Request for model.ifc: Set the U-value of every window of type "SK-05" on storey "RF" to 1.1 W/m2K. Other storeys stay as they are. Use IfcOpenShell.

First a look at what the model holds.

```python
import ifcopenshell
import ifcopenshell.util.element

model = ifcopenshell.open("model.ifc")
print(model.schema)
storey = next(s for s in model.by_type("IfcBuildingStorey") if s.Name == "RF")
windows = [e for e in ifcopenshell.util.element.get_decomposition(storey) if e.is_a("IfcWindow")]
seen = {}
for e in windows:
    element_type = ifcopenshell.util.element.get_type(e)
    key = (element_type.Name if element_type != e and element_type else None, ifcopenshell.util.element.get_pset(e, "Pset_WindowCommon", "ThermalTransmittance"))
    seen[key] = seen.get(key, 0) + 1
for (name, value), count in sorted(seen.items(), key=str):
    print(count, "x", name, "|", value)
```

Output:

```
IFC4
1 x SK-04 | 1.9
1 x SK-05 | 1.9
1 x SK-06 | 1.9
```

```python
import ifcopenshell
import ifcopenshell.api.pset
import ifcopenshell.util.element

model = ifcopenshell.open("model.ifc")

storey = next(s for s in model.by_type("IfcBuildingStorey") if s.Name == "RF")
windows = [e for e in ifcopenshell.util.element.get_decomposition(storey) if e.is_a("IfcWindow")]

count = 0
for e in windows:
    element_type = ifcopenshell.util.element.get_type(e)
    if element_type in (None, e) or element_type.Name != "SK-05":
        continue
    # add_pset returns the element's existing set when there is one.
    pset = ifcopenshell.api.pset.add_pset(model, product=e, name="Pset_WindowCommon")
    ifcopenshell.api.pset.edit_pset(model, pset=pset, properties={"ThermalTransmittance": 1.1})
    count += 1

print(count, "windows updated")

model.write("model_edited.ifc")
```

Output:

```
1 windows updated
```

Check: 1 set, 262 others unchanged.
